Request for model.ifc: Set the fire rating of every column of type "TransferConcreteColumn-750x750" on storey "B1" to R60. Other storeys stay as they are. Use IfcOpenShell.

First a look at what the model holds.

```python
import ifcopenshell
import ifcopenshell.util.element

model = ifcopenshell.open("model.ifc")
print(model.schema)
storey = next(s for s in model.by_type("IfcBuildingStorey") if s.Name == "B1")
columns = [e for e in ifcopenshell.util.element.get_decomposition(storey) if e.is_a("IfcColumn")]
seen = {}
for e in columns:
    element_type = ifcopenshell.util.element.get_type(e)
    key = (element_type.Name if element_type != e and element_type else None, ifcopenshell.util.element.get_pset(e, "Pset_ColumnCommon", "FireRating"))
    seen[key] = seen.get(key, 0) + 1
for (name, value), count in sorted(seen.items(), key=str):
    print(count, "x", name, "|", value)
```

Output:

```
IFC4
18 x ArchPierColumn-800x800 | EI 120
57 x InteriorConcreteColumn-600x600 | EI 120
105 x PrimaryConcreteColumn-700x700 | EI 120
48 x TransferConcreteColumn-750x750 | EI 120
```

```python
import ifcopenshell
import ifcopenshell.api.pset
import ifcopenshell.util.element

model = ifcopenshell.open("model.ifc")

storey = next(s for s in model.by_type("IfcBuildingStorey") if s.Name == "B1")
columns = [e for e in ifcopenshell.util.element.get_decomposition(storey) if e.is_a("IfcColumn")]

count = 0
for e in columns:
    element_type = ifcopenshell.util.element.get_type(e)
    if element_type in (None, e) or element_type.Name != "TransferConcreteColumn-750x750":
        continue
    # add_pset returns the element's existing set when there is one.
    pset = ifcopenshell.api.pset.add_pset(model, product=e, name="Pset_ColumnCommon")
    ifcopenshell.api.pset.edit_pset(model, pset=pset, properties={"FireRating": "R60"})
    count += 1

print(count, "columns updated")

model.write("model_v2.ifc")
```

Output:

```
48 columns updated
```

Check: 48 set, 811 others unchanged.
